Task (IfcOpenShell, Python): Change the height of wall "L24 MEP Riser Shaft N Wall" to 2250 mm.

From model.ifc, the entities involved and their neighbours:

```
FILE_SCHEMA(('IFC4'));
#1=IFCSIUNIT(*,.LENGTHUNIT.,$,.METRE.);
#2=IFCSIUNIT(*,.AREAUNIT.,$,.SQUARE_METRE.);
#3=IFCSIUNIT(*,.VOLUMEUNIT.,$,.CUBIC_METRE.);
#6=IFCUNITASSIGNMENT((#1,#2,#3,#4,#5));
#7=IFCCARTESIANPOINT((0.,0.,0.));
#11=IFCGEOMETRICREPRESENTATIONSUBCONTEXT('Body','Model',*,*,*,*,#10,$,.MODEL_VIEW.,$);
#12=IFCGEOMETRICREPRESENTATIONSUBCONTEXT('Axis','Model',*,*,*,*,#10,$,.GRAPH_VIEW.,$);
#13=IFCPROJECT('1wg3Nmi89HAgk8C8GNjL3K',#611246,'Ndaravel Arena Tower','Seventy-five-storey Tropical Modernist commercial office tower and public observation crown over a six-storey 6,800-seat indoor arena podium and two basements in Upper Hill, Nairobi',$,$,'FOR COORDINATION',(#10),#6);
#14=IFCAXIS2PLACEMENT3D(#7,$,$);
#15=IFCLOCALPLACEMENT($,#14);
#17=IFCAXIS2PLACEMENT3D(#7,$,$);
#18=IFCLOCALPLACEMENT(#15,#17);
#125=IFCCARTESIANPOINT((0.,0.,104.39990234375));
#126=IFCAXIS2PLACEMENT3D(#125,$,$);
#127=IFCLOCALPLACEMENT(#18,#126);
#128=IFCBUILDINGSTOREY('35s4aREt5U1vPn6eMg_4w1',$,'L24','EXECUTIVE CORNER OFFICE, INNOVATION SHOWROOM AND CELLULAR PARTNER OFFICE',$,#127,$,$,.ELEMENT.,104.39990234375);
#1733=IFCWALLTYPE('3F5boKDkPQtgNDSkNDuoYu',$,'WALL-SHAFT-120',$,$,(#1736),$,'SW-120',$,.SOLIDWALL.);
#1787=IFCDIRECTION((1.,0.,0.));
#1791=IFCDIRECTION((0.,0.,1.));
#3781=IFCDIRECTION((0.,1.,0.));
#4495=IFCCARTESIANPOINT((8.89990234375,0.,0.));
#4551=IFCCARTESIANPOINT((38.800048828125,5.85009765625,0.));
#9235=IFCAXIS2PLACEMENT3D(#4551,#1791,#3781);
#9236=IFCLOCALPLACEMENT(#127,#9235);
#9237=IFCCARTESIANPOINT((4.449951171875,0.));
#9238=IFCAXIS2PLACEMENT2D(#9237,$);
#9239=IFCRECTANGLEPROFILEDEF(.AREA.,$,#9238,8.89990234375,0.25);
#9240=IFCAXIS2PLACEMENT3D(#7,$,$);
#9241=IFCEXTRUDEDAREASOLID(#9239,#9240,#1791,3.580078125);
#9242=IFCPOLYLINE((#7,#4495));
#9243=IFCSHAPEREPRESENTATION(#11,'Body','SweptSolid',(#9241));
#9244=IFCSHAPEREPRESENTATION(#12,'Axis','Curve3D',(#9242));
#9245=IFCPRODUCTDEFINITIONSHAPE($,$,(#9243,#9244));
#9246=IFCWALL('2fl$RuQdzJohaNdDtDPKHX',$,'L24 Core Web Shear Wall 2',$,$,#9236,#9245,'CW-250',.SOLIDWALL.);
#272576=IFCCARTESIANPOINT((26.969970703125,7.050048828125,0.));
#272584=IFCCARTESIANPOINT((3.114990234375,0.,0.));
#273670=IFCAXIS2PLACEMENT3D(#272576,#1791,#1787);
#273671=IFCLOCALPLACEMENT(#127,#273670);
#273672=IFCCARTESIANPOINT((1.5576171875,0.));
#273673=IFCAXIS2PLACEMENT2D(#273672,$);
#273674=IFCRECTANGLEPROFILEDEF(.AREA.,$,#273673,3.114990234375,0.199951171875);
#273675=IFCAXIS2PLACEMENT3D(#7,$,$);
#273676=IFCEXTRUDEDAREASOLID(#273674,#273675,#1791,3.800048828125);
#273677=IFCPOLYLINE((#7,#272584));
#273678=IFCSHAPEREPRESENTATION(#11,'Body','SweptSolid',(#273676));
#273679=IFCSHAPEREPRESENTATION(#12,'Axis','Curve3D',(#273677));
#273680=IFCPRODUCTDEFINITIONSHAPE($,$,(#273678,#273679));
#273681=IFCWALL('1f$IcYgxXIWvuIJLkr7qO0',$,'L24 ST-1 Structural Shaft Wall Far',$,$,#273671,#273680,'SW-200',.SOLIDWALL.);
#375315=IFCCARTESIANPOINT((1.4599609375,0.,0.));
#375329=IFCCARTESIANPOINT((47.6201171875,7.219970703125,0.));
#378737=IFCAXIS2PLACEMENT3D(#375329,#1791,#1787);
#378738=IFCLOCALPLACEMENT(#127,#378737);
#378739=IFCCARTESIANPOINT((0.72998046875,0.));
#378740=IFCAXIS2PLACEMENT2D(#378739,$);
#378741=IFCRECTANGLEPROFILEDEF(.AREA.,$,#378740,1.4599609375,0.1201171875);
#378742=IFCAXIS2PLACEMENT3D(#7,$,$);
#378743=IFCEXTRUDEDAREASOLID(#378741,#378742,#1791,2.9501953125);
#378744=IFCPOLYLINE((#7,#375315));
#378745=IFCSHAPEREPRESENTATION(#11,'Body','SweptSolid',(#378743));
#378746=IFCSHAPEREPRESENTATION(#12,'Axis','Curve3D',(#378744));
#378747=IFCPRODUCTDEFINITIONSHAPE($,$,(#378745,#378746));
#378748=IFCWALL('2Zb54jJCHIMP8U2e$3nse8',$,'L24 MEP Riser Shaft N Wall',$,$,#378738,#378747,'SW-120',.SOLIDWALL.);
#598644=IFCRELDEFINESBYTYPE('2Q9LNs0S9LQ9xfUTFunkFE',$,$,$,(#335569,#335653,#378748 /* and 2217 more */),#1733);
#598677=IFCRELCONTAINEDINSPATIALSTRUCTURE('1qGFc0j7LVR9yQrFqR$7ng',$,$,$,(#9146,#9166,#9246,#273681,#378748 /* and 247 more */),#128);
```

```python
import ifcopenshell
import ifcopenshell.geom
import ifcopenshell.util.representation
import ifcopenshell.util.shape

model = ifcopenshell.open("model.ifc")
settings = ifcopenshell.geom.settings()


def volume(element):
    """Net volume in cubic metres, openings subtracted."""
    shape = ifcopenshell.geom.create_shape(settings, element)
    return ifcopenshell.util.shape.get_volume(shape.geometry)


wall = model.by_id(378748)
before = volume(wall)

body = ifcopenshell.util.representation.get_representation(wall, "Model", "Body")
solid = body.Items[0]
old_height = solid.Depth
solid.Depth = 2.25
after = volume(wall)

print(f"height {old_height:g} -> {solid.Depth:g}, volume {before:.3f} -> {after:.3f} m3")

model.write("model-out.ifc")
```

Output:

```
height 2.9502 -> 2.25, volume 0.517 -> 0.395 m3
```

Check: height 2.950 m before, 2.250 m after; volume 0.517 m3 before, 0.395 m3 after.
